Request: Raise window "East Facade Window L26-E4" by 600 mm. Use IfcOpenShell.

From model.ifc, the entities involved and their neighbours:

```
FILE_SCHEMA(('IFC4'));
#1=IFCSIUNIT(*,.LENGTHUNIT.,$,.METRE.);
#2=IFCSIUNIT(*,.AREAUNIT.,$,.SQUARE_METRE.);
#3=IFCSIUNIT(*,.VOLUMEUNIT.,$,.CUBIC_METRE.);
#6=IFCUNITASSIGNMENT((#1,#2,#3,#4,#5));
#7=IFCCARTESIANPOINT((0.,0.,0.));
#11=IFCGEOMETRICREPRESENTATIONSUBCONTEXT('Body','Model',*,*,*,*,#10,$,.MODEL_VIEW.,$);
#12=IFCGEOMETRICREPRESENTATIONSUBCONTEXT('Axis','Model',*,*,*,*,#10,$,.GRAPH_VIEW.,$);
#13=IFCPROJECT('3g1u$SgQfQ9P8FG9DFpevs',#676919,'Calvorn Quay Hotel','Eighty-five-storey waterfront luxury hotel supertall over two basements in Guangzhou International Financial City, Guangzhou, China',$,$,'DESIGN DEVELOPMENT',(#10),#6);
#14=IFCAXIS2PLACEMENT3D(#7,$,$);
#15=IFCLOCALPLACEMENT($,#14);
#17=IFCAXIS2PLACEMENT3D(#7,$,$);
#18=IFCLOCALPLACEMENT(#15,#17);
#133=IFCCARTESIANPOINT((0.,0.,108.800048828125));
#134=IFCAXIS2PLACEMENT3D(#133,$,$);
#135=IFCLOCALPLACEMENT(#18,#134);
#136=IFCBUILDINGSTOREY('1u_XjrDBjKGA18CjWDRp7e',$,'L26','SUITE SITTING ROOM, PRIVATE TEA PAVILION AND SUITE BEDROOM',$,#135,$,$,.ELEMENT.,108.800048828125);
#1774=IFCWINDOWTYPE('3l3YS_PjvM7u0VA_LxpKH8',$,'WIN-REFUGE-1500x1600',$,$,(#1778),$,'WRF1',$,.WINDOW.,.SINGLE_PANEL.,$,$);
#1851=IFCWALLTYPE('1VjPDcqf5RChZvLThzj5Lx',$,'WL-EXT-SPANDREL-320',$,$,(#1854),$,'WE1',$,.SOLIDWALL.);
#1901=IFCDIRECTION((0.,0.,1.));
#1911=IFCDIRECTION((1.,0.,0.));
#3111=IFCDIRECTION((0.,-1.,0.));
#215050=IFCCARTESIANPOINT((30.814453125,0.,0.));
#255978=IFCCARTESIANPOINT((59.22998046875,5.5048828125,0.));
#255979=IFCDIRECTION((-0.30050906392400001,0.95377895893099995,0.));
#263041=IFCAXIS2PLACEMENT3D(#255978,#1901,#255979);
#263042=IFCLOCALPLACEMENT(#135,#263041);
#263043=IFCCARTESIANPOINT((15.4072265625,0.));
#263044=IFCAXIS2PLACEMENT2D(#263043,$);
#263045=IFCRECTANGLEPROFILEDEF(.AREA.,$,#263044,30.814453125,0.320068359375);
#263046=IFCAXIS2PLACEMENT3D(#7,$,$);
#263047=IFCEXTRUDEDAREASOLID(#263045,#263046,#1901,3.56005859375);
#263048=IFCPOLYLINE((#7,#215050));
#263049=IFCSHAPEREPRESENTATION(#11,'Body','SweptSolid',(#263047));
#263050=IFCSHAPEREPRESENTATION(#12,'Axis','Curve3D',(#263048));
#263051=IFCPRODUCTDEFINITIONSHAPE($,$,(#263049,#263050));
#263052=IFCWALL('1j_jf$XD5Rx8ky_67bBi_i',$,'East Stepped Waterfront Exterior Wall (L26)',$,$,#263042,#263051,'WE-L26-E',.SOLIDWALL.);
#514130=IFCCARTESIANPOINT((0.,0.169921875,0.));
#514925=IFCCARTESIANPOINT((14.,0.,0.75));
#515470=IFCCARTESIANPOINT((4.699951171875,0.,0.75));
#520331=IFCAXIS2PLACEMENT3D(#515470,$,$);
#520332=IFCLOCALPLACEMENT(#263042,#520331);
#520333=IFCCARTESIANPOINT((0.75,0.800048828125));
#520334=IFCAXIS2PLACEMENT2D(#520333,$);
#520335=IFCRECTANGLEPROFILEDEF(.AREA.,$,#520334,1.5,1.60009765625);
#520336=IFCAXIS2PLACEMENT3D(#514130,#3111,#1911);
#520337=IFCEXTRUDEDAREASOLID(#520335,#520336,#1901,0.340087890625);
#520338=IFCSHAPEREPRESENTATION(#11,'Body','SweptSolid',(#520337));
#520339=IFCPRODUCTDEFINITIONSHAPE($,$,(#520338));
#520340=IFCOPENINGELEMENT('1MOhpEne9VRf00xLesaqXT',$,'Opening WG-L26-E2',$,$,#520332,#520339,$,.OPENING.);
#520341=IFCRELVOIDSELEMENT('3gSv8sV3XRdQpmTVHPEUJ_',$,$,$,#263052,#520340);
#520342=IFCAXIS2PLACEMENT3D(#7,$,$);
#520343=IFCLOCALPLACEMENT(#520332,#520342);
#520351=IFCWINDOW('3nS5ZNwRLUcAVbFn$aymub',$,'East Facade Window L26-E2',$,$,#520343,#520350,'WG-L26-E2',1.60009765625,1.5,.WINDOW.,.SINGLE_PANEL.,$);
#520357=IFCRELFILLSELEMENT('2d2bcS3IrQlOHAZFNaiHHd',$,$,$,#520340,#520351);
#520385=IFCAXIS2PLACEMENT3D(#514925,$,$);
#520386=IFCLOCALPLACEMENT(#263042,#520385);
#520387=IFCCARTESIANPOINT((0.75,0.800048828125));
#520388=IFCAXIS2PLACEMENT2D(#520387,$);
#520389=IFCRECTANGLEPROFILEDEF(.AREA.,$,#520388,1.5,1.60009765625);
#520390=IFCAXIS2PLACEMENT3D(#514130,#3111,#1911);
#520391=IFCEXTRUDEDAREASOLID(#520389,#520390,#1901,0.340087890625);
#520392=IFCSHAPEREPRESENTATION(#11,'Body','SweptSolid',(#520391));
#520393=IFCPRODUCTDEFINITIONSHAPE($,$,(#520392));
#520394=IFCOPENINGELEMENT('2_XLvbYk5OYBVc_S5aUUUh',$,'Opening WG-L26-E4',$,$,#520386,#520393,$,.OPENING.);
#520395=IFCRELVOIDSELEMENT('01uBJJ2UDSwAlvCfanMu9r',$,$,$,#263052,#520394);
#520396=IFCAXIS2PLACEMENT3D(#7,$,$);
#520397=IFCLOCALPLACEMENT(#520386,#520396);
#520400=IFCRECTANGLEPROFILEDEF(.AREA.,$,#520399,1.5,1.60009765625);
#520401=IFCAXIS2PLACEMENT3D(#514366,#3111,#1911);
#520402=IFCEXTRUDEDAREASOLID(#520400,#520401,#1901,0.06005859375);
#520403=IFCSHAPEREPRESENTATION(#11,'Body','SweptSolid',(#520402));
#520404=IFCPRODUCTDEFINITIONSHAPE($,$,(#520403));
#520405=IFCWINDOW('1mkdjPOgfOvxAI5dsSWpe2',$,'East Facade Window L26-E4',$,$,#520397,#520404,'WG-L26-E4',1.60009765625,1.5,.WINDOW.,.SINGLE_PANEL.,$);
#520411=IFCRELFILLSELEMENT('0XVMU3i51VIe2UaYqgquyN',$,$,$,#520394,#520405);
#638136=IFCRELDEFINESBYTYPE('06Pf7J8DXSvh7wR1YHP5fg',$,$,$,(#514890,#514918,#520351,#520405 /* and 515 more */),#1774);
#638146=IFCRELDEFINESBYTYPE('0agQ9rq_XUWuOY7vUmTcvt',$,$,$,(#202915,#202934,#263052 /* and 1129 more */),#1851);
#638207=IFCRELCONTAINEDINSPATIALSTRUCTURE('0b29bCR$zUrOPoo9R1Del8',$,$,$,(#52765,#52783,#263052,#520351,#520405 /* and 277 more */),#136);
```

```python
import numpy as np
import ifcopenshell
import ifcopenshell.api.geometry
import ifcopenshell.util.placement
import ifcopenshell.util.unit

model = ifcopenshell.open("model.ifc")
unit_scale = ifcopenshell.util.unit.calculate_unit_scale(model)

window = model.by_id(520405)
opening = window.FillsVoids[0].RelatingOpeningElement
dz = 0.6 / unit_scale

shift = np.array([0.0, 0.0, dz])
# The window is placed relative to its opening, so it follows when the opening moves.
matrix = ifcopenshell.util.placement.get_local_placement(opening.ObjectPlacement)
matrix[:3, 3] += shift
ifcopenshell.api.geometry.edit_object_placement(
    model, product=opening, matrix=matrix, is_si=False, should_transform_children=True
)

print(f"moved by {dz * unit_scale:+.3f} m")

model.write("model_edited.ifc")
```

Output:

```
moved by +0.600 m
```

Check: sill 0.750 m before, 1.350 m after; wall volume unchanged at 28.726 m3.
